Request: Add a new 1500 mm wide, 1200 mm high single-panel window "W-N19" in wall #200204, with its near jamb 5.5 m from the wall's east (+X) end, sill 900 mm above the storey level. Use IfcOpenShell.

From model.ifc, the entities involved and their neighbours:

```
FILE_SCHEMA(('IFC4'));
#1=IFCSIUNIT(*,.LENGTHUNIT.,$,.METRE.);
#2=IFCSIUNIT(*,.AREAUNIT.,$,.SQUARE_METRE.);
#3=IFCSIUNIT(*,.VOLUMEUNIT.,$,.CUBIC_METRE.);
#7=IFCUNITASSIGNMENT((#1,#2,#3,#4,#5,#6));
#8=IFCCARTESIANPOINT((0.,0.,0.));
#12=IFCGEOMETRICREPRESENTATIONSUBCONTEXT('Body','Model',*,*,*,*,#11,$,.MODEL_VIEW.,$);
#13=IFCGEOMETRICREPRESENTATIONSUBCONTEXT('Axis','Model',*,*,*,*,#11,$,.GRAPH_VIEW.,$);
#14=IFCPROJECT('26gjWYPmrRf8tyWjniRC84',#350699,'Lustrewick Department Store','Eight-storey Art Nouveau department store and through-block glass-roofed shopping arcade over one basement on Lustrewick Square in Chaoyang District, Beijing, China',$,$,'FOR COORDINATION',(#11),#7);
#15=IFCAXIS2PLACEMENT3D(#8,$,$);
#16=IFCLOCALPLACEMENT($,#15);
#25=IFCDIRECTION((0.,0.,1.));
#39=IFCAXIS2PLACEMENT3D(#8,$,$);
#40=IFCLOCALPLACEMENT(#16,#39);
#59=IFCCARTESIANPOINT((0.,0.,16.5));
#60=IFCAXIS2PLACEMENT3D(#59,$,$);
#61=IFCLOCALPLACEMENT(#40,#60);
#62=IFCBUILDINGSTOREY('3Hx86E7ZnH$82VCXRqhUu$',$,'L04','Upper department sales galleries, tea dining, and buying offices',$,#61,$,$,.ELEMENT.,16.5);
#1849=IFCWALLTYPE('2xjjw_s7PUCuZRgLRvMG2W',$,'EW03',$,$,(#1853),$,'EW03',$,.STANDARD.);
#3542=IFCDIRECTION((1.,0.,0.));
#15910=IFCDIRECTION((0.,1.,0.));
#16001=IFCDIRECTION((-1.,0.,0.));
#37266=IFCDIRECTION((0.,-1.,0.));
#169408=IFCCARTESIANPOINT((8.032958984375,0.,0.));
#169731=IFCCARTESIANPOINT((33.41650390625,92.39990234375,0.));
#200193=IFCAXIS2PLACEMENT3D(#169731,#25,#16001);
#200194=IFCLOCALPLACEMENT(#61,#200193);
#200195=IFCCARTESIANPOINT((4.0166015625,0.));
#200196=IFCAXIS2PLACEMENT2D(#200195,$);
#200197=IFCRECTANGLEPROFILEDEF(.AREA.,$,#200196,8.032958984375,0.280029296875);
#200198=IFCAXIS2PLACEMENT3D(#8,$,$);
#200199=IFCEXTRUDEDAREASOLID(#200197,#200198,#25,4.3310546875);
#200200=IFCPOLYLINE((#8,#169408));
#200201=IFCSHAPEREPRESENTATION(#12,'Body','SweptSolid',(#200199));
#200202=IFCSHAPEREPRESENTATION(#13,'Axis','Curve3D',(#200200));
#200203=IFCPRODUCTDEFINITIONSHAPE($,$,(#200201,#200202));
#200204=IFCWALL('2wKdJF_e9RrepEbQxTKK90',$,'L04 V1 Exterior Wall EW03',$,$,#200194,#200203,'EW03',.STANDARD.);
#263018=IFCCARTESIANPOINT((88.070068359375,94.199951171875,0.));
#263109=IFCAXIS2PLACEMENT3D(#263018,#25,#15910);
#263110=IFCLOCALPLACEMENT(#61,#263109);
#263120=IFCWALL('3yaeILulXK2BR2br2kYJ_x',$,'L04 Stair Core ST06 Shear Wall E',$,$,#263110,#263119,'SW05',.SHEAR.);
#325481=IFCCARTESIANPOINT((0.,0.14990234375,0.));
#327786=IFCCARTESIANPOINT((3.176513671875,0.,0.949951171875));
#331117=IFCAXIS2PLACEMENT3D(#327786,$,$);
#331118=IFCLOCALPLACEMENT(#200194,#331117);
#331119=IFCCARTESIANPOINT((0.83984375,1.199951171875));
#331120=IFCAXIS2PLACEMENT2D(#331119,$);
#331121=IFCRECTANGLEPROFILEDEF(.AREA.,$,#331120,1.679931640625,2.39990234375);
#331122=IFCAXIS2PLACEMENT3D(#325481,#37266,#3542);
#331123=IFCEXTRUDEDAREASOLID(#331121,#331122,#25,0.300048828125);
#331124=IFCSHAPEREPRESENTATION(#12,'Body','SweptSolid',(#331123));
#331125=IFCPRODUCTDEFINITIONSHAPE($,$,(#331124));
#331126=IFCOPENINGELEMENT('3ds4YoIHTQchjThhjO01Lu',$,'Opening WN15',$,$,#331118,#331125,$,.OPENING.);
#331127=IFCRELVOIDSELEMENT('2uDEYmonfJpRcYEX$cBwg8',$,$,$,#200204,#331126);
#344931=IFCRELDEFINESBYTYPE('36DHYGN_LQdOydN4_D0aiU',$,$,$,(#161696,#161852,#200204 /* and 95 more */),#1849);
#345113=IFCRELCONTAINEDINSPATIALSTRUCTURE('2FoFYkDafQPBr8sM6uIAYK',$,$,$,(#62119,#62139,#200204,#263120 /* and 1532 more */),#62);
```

```python
import numpy as np
import ifcopenshell
import ifcopenshell.api.feature
import ifcopenshell.api.geometry
import ifcopenshell.api.root
import ifcopenshell.api.spatial
import ifcopenshell.geom
import ifcopenshell.util.element
import ifcopenshell.util.placement
import ifcopenshell.util.representation
import ifcopenshell.util.shape
import ifcopenshell.util.unit

model = ifcopenshell.open("model.ifc")
unit_scale = ifcopenshell.util.unit.calculate_unit_scale(model)
settings = ifcopenshell.geom.settings()


def volume(element):
    """Net volume in cubic metres, openings subtracted."""
    shape = ifcopenshell.geom.create_shape(settings, element)
    return ifcopenshell.util.shape.get_volume(shape.geometry)


wall = model.by_guid("2wKdJF_e9RrepEbQxTKK90")
storey = ifcopenshell.util.element.get_container(wall, ifc_class="IfcBuildingStorey")
context = ifcopenshell.util.representation.get_context(model, "Model", "Body", "MODEL_VIEW")
before = volume(wall)

width, height, from_end, sill = 1.5, 1.2, 5.5, 0.9  # metres

# The wall runs along its own X axis, and the end named is its -X end.
wall_shape = ifcopenshell.geom.create_shape(settings, wall)
x, y, z = ifcopenshell.util.shape.get_vertices(wall_shape.geometry).T
start = x.min() + from_end
face, thickness = float(y.min()), float(y.max() - y.min())
wall_matrix = ifcopenshell.util.placement.get_local_placement(wall.ObjectPlacement)
level = ifcopenshell.util.placement.get_local_placement(storey.ObjectPlacement)[2, 3]


def in_wall(x, y):
    """Placement at x, y metres in the wall's axes, at sill height."""
    matrix = wall_matrix.copy()
    matrix[:, 3] = wall_matrix @ np.array([x / unit_scale, y / unit_scale, 0.0, 1.0])
    matrix[2, 3] = level + sill / unit_scale
    return matrix


# Opening: a box that overshoots both wall faces by 50 mm.
opening = ifcopenshell.api.root.create_entity(model, ifc_class="IfcOpeningElement", predefined_type="OPENING")
box = ifcopenshell.api.geometry.add_wall_representation(
    model, context=context, length=width, height=height, thickness=thickness + 0.1
)
ifcopenshell.api.geometry.assign_representation(model, product=opening, representation=box)
ifcopenshell.api.geometry.edit_object_placement(model, product=opening, matrix=in_wall(start, face - 0.05), is_si=False)
ifcopenshell.api.feature.add_feature(model, feature=opening, element=wall)

window = ifcopenshell.api.root.create_entity(model, ifc_class="IfcWindow", name="W-N19", predefined_type="WINDOW")
window.OverallWidth, window.OverallHeight = width / unit_scale, height / unit_scale
window.PartitioningType = "SINGLE_PANEL"
body = ifcopenshell.api.geometry.add_window_representation(
    model,
    context=context,
    overall_width=window.OverallWidth,
    overall_height=window.OverallHeight,
    partition_type="SINGLE_PANEL",
)
ifcopenshell.api.geometry.assign_representation(model, product=window, representation=body)
ifcopenshell.api.spatial.assign_container(model, products=[window], relating_structure=storey)
ifcopenshell.api.feature.add_filling(model, opening=opening, element=window)

# Centre the window in the wall's thickness.
ifcopenshell.api.geometry.edit_object_placement(model, product=window, matrix=in_wall(start, face), is_si=False)
window_shape = ifcopenshell.geom.create_shape(settings, window)
depth = ifcopenshell.util.shape.get_vertices(window_shape.geometry)[:, 1]
offset = face + thickness / 2 - (depth.min() + depth.max()) / 2
ifcopenshell.api.geometry.edit_object_placement(model, product=window, matrix=in_wall(start, offset), is_si=False)

after = volume(wall)

print(f"wall volume {before:.3f} -> {after:.3f} m3")

model.write("model_updated.ifc")
```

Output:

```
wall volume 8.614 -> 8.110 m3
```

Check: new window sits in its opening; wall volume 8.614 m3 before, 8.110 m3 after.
